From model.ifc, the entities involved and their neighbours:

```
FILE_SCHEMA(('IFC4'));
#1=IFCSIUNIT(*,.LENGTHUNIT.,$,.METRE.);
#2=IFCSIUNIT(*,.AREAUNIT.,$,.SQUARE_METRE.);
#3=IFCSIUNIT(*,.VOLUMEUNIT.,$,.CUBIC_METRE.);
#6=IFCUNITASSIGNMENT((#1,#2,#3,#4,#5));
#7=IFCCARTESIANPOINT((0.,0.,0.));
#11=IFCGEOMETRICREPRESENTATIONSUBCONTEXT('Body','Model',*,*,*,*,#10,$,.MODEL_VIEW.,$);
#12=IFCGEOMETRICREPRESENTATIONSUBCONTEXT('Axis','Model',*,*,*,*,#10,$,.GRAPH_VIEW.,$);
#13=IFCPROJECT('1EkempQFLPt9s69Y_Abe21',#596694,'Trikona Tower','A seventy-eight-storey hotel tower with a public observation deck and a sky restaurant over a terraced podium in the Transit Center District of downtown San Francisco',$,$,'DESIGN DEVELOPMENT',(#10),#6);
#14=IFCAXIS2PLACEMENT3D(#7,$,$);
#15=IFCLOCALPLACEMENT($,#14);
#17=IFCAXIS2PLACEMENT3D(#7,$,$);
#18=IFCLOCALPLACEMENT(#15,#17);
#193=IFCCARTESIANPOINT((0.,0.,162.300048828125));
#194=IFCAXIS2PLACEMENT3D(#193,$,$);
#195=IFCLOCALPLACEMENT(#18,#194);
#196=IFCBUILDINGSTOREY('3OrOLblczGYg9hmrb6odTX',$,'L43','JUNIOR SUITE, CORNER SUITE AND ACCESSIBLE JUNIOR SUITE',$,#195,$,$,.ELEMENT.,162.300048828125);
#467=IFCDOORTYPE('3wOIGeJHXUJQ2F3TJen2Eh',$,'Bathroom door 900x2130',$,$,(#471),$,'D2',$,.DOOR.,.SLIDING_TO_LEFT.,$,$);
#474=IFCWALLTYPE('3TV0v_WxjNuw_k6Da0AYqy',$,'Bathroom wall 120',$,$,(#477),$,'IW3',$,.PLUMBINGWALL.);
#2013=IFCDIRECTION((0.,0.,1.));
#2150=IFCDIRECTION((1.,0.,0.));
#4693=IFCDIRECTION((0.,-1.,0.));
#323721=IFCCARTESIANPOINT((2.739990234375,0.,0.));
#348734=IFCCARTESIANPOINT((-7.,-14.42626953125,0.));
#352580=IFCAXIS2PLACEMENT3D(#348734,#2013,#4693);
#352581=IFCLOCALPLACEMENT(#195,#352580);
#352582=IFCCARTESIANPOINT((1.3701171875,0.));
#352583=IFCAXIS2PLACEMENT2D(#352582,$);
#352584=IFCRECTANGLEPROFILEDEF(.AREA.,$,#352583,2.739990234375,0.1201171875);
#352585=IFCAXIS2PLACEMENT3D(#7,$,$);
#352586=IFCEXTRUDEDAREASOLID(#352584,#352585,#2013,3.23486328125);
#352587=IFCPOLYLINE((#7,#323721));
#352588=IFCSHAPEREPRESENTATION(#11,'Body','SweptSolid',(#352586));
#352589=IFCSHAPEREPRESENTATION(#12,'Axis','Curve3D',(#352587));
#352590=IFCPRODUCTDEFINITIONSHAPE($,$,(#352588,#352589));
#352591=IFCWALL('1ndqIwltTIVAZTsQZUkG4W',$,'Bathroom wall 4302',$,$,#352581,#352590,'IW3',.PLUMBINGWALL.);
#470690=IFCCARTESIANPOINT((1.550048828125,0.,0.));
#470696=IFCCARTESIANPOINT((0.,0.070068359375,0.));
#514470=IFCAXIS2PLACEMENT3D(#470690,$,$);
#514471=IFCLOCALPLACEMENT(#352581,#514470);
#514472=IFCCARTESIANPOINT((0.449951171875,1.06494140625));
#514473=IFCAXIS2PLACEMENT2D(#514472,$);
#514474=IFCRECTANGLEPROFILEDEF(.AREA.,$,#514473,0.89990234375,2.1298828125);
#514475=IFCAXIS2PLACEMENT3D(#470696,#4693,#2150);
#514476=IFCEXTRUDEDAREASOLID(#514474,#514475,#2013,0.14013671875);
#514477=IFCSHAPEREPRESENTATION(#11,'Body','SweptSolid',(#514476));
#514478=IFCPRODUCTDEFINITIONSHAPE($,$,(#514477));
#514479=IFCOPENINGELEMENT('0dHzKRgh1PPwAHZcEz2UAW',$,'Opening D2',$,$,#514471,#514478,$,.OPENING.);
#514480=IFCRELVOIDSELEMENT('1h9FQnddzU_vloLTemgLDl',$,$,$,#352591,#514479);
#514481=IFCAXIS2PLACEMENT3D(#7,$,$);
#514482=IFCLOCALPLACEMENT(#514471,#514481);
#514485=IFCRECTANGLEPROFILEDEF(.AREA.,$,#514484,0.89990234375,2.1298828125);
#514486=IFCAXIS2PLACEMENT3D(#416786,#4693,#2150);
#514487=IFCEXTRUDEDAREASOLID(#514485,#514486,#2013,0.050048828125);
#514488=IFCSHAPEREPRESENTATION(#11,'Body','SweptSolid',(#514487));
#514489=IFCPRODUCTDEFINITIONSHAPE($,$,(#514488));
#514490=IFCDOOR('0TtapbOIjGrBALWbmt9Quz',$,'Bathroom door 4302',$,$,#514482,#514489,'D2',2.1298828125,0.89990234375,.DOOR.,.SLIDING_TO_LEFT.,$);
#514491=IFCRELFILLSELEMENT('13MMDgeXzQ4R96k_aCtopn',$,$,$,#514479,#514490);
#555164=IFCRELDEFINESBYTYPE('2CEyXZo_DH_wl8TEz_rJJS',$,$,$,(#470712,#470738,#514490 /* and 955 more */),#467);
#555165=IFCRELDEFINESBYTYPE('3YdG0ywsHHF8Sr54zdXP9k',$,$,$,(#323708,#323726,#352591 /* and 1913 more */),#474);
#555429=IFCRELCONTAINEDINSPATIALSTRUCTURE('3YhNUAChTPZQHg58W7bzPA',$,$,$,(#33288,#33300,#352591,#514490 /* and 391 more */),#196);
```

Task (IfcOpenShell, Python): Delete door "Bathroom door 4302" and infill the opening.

```python
import ifcopenshell
import ifcopenshell.api.feature
import ifcopenshell.api.root
import ifcopenshell.geom
import ifcopenshell.util.shape

model = ifcopenshell.open("model.ifc")
settings = ifcopenshell.geom.settings()


def volume(element):
    """Net volume in cubic metres, openings subtracted."""
    shape = ifcopenshell.geom.create_shape(settings, element)
    return ifcopenshell.util.shape.get_volume(shape.geometry)


door = model.by_guid("0TtapbOIjGrBALWbmt9Quz")
opening = door.FillsVoids[0].RelatingOpeningElement
wall = opening.VoidsElements[0].RelatingBuildingElement
before = volume(wall)

ifcopenshell.api.root.remove_product(model, product=door)
ifcopenshell.api.feature.remove_feature(model, feature=opening)

after = volume(wall)

print(f"wall volume {before:.3f} -> {after:.3f} m3")

model.write("model-out.ifc")
```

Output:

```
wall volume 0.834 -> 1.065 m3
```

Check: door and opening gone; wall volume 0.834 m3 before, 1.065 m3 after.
